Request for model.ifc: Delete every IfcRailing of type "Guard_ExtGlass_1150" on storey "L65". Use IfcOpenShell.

First a look at what the model holds.

```python
import ifcopenshell
import ifcopenshell.util.element

model = ifcopenshell.open("model.ifc")
print(model.schema)
storey = next(s for s in model.by_type("IfcBuildingStorey") if s.Name == "L65")
railings = [e for e in ifcopenshell.util.element.get_decomposition(storey) if e.is_a("IfcRailing")]
seen = {}
for e in railings:
    element_type = ifcopenshell.util.element.get_type(e)
    name = element_type.Name if element_type not in (None, e) else None
    seen[name] = seen.get(name, 0) + 1
for name, count in sorted(seen.items(), key=str):
    print(count, "x", name)
```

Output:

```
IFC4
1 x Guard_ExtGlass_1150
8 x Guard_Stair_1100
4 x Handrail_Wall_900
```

```python
import ifcopenshell
import ifcopenshell.api.root
import ifcopenshell.util.element

model = ifcopenshell.open("model.ifc")

storey = next(s for s in model.by_type("IfcBuildingStorey") if s.Name == "L65")
railings = [e for e in ifcopenshell.util.element.get_decomposition(storey) if e.is_a("IfcRailing")]
targets = [e for e in railings if (t := ifcopenshell.util.element.get_type(e)) not in (None, e) and t.Name == "Guard_ExtGlass_1150"]

for e in targets:
    ifcopenshell.api.root.remove_product(model, product=e)
print(len(targets), "removed")

model.write("model-out.ifc")
```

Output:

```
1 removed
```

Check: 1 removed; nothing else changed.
